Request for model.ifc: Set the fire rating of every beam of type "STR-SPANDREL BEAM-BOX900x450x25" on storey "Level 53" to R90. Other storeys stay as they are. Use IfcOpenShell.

First a look at what the model holds.

```python
import ifcopenshell
import ifcopenshell.util.element

model = ifcopenshell.open("model.ifc")
print(model.schema)
storey = next(s for s in model.by_type("IfcBuildingStorey") if s.Name == "Level 53")
beams = [e for e in ifcopenshell.util.element.get_decomposition(storey) if e.is_a("IfcBeam")]
seen = {}
for e in beams:
    element_type = ifcopenshell.util.element.get_type(e)
    key = (element_type.Name if element_type != e and element_type else None, ifcopenshell.util.element.get_pset(e, "Pset_BeamCommon", "FireRating"))
    seen[key] = seen.get(key, 0) + 1
for (name, value), count in sorted(seen.items(), key=str):
    print(count, "x", name, "|", value)
```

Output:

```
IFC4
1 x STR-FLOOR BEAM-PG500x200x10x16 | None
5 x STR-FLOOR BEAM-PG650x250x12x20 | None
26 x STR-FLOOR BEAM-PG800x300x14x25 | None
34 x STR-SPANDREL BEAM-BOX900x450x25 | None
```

```python
import ifcopenshell
import ifcopenshell.api.pset
import ifcopenshell.util.element

model = ifcopenshell.open("model.ifc")

storey = next(s for s in model.by_type("IfcBuildingStorey") if s.Name == "Level 53")
beams = [e for e in ifcopenshell.util.element.get_decomposition(storey) if e.is_a("IfcBeam")]

count = 0
for e in beams:
    element_type = ifcopenshell.util.element.get_type(e)
    if element_type in (None, e) or element_type.Name != "STR-SPANDREL BEAM-BOX900x450x25":
        continue
    found = ifcopenshell.util.element.get_pset(e, "Pset_BeamCommon", should_inherit=False)
    if found:
        pset = model.by_id(found["id"])
        if len(ifcopenshell.util.element.get_elements_by_pset(pset)) > 1:
            pset = ifcopenshell.api.pset.unshare_pset(model, products=[e], pset=pset)[0]
    else:
        pset = ifcopenshell.api.pset.add_pset(model, product=e, name="Pset_BeamCommon")
    ifcopenshell.api.pset.edit_pset(model, pset=pset, properties={"FireRating": "R90"})
    count += 1

print(count, "beams updated")

model.write("model_updated.ifc")
```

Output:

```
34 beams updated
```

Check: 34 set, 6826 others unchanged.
